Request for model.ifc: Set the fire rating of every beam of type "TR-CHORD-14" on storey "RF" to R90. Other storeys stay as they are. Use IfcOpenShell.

First a look at what the model holds.

```python
import ifcopenshell
import ifcopenshell.util.element

model = ifcopenshell.open("model.ifc")
print(model.schema)
storey = next(s for s in model.by_type("IfcBuildingStorey") if s.Name == "RF")
beams = [e for e in ifcopenshell.util.element.get_decomposition(storey) if e.is_a("IfcBeam")]
seen = {}
for e in beams:
    element_type = ifcopenshell.util.element.get_type(e)
    key = (element_type.Name if element_type != e and element_type else None, ifcopenshell.util.element.get_pset(e, "Pset_BeamCommon", "FireRating"))
    seen[key] = seen.get(key, 0) + 1
for (name, value), count in sorted(seen.items(), key=str):
    print(count, "x", name, "|", value)
```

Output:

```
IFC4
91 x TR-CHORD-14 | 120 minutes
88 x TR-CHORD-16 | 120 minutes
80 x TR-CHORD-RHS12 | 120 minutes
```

```python
import ifcopenshell
import ifcopenshell.api.pset
import ifcopenshell.util.element

model = ifcopenshell.open("model.ifc")

storey = next(s for s in model.by_type("IfcBuildingStorey") if s.Name == "RF")
beams = [e for e in ifcopenshell.util.element.get_decomposition(storey) if e.is_a("IfcBeam")]

count = 0
for e in beams:
    element_type = ifcopenshell.util.element.get_type(e)
    if element_type in (None, e) or element_type.Name != "TR-CHORD-14":
        continue
    # add_pset returns the element's existing set when there is one.
    pset = ifcopenshell.api.pset.add_pset(model, product=e, name="Pset_BeamCommon")
    ifcopenshell.api.pset.edit_pset(model, pset=pset, properties={"FireRating": "R90"})
    count += 1

print(count, "beams updated")

model.write("model_rev.ifc")
```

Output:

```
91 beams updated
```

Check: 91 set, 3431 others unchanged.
